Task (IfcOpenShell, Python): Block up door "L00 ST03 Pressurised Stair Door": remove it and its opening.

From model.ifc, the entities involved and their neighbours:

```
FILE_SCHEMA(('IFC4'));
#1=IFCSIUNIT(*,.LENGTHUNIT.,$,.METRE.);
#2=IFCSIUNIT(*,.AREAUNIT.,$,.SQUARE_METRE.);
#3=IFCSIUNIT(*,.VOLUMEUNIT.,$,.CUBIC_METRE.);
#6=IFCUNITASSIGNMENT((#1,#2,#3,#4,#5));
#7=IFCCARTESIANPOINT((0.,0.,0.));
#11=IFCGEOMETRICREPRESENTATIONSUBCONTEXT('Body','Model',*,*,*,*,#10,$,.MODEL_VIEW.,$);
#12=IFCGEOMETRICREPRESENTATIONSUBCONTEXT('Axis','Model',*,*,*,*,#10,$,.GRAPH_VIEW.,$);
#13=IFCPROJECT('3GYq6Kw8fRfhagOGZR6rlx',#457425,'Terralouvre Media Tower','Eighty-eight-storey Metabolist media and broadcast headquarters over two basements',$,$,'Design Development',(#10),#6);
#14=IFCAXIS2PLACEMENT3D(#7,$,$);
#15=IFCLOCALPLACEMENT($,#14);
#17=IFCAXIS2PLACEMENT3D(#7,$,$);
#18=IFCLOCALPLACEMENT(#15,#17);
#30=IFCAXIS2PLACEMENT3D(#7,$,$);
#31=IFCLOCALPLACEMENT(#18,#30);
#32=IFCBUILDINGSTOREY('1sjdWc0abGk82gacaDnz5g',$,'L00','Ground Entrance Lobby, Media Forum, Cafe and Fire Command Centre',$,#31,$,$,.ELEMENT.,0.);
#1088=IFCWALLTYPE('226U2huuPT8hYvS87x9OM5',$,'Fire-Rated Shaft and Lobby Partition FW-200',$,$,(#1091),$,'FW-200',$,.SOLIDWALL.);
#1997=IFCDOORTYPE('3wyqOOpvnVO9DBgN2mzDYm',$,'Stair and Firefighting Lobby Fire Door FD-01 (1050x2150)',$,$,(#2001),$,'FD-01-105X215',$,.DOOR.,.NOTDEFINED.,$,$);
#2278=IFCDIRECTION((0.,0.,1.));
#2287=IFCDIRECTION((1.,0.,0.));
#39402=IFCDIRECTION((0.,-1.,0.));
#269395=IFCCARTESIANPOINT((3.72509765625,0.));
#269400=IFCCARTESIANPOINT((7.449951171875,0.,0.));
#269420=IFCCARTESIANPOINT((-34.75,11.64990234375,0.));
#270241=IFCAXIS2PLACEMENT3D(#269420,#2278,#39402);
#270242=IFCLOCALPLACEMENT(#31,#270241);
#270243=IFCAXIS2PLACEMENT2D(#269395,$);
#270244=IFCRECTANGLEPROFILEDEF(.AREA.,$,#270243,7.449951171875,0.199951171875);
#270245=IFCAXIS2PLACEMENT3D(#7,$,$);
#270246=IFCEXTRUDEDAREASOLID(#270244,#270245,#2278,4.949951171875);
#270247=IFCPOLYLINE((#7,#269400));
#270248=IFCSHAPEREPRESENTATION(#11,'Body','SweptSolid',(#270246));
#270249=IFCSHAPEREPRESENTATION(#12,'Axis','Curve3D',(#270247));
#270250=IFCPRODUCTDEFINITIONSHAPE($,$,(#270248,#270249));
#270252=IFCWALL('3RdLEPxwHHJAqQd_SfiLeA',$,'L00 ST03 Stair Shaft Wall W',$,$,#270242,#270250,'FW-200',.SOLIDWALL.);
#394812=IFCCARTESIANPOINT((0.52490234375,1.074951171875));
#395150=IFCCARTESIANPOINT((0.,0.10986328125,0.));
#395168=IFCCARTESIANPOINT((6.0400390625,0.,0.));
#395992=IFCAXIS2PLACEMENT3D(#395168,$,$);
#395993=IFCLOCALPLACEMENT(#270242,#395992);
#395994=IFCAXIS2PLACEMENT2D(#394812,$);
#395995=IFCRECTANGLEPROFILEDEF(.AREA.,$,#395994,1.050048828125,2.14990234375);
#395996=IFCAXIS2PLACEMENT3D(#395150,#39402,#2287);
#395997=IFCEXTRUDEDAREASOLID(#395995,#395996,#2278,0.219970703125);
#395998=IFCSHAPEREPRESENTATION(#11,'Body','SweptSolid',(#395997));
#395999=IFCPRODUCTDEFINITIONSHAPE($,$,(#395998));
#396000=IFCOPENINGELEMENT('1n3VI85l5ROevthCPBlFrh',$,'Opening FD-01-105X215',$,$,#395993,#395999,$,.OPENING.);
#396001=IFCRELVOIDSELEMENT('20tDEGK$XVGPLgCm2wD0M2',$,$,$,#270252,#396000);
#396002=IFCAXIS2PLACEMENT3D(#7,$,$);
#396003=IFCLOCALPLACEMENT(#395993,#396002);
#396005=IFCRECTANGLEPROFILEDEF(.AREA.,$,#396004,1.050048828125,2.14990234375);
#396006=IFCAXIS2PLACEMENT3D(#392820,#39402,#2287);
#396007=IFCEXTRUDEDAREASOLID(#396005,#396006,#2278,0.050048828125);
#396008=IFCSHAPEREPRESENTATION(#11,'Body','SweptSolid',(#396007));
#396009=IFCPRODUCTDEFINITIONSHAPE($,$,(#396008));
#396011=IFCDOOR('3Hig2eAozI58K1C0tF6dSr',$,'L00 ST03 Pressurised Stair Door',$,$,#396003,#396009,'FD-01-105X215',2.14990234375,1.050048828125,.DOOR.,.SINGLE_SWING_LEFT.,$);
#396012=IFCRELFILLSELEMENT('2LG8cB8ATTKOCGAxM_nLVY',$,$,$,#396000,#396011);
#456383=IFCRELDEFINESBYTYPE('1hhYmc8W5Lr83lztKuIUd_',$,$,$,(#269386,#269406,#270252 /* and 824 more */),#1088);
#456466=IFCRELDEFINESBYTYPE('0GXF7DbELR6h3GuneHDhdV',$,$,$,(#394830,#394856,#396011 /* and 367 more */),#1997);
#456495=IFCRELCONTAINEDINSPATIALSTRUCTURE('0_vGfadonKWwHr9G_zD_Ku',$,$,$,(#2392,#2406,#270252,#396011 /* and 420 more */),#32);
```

```python
import ifcopenshell
import ifcopenshell.api.feature
import ifcopenshell.api.root
import ifcopenshell.geom
import ifcopenshell.util.shape

model = ifcopenshell.open("model.ifc")
settings = ifcopenshell.geom.settings()


def volume(element):
    """Net volume in cubic metres, openings subtracted."""
    shape = ifcopenshell.geom.create_shape(settings, element)
    return ifcopenshell.util.shape.get_volume(shape.geometry)


door = model.by_id(396011)
opening = door.FillsVoids[0].RelatingOpeningElement
wall = opening.VoidsElements[0].RelatingBuildingElement
before = volume(wall)

ifcopenshell.api.root.remove_product(model, product=door)
ifcopenshell.api.feature.remove_feature(model, feature=opening)

after = volume(wall)

print(f"wall volume {before:.3f} -> {after:.3f} m3")

model.write("model-out.ifc")
```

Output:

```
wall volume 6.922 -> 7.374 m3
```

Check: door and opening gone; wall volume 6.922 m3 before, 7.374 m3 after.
